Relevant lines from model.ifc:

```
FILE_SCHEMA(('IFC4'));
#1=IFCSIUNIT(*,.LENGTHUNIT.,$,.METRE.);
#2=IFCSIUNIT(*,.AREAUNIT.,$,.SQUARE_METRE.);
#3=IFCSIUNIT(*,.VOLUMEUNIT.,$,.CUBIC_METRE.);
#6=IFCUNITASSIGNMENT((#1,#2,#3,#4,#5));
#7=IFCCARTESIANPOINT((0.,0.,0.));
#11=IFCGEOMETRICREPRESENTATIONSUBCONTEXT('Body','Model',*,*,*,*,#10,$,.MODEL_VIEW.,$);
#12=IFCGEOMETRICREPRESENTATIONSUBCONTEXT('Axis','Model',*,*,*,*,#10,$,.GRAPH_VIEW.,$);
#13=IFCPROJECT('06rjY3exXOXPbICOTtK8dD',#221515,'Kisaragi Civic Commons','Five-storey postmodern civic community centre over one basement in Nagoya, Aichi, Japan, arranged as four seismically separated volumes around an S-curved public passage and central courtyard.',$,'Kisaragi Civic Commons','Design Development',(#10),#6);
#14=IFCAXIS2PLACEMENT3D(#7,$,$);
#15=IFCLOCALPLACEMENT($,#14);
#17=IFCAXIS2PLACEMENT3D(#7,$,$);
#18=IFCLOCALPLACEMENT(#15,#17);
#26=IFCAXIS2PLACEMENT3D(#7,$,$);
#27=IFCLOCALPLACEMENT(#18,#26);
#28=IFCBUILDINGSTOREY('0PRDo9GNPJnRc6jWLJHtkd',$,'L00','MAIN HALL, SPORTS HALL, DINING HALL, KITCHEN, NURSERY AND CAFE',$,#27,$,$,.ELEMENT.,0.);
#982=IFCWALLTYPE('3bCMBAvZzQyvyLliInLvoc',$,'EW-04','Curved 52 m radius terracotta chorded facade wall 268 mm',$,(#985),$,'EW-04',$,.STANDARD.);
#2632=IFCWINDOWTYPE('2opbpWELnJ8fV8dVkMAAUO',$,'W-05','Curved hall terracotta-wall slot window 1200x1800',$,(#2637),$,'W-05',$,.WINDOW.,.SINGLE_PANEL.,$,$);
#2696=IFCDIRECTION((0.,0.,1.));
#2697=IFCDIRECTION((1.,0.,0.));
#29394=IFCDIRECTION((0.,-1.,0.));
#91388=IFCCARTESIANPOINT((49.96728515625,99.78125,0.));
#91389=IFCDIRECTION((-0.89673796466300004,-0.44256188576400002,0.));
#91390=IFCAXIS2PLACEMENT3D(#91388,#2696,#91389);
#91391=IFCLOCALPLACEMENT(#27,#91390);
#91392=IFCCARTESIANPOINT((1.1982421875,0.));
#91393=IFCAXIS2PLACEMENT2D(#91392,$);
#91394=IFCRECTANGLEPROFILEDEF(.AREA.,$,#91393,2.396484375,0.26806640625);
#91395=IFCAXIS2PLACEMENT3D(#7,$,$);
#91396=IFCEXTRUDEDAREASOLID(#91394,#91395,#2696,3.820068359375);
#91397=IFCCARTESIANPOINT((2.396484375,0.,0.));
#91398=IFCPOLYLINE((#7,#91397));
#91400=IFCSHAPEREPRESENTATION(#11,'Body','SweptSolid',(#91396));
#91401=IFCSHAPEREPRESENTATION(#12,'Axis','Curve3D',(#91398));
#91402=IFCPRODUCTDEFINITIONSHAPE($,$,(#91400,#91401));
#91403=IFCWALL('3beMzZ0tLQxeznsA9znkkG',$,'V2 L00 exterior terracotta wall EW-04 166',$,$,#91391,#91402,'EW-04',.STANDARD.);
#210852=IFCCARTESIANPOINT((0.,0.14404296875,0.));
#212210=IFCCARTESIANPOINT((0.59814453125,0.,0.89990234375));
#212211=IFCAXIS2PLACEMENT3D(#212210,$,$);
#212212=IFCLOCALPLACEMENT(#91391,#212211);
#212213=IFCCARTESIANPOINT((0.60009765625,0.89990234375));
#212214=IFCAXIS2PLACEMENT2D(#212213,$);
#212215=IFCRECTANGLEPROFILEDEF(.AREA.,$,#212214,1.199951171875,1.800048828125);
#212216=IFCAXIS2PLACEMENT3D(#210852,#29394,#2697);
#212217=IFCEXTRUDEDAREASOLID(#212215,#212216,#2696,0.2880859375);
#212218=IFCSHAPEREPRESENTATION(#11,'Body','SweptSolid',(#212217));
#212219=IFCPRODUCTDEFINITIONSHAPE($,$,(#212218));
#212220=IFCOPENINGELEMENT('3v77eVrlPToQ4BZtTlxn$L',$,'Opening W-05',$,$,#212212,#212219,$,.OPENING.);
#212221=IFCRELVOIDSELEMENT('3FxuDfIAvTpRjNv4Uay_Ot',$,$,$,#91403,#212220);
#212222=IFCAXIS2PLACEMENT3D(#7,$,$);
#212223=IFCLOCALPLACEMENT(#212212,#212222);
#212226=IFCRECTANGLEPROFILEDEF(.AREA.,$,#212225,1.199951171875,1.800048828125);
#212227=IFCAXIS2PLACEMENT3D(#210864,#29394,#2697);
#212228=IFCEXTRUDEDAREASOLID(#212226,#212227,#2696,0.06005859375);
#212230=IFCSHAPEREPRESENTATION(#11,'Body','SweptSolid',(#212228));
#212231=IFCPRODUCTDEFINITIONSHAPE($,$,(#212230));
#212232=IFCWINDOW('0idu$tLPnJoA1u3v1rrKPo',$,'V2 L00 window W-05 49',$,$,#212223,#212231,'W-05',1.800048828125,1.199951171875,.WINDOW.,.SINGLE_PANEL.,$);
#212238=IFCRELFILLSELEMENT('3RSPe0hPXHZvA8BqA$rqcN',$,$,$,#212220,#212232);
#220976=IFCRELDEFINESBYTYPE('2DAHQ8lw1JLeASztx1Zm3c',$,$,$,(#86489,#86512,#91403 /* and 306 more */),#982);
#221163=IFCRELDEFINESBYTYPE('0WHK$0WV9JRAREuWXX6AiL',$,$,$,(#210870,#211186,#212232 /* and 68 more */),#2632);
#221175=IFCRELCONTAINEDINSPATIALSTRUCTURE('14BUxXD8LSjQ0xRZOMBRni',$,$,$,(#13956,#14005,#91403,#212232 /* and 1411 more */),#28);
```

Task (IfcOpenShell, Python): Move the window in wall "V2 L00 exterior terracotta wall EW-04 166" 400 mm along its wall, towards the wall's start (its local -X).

```python
import ifcopenshell
import ifcopenshell.api.geometry
import ifcopenshell.util.placement
import ifcopenshell.util.unit

model = ifcopenshell.open("model.ifc")
unit_scale = ifcopenshell.util.unit.calculate_unit_scale(model)

window = model.by_guid("0idu$tLPnJoA1u3v1rrKPo")
opening = window.FillsVoids[0].RelatingOpeningElement
wall = opening.VoidsElements[0].RelatingBuildingElement

wall_matrix = ifcopenshell.util.placement.get_local_placement(wall.ObjectPlacement)
shift = wall_matrix[:3, 0] * -0.4 / unit_scale
before = ifcopenshell.util.placement.get_local_placement(window.ObjectPlacement)[:3, 3].copy()

# The window is placed relative to its opening, so it follows when the opening moves.
matrix = ifcopenshell.util.placement.get_local_placement(opening.ObjectPlacement)
matrix[:3, 3] += shift
ifcopenshell.api.geometry.edit_object_placement(
    model, product=opening, matrix=matrix, is_si=False, should_transform_children=True
)

after = ifcopenshell.util.placement.get_local_placement(window.ObjectPlacement)[:3, 3]
print("window moved by", (after - before).round(3) + 0.0)

model.write("model_updated.ifc")
```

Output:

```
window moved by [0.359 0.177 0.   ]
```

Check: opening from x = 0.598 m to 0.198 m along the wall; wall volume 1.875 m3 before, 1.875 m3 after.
